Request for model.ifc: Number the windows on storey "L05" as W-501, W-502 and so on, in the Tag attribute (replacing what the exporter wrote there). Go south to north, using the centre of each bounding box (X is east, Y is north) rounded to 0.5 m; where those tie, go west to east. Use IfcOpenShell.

First a look at what the model holds.

```python
import ifcopenshell
import ifcopenshell.util.element
import ifcopenshell.util.placement

model = ifcopenshell.open("model.ifc")
print(model.schema)
storey = next(s for s in model.by_type("IfcBuildingStorey") if s.Name == "L05")
windows = [e for e in ifcopenshell.util.element.get_decomposition(storey) if e.is_a("IfcWindow")]
for e in sorted(windows, key=lambda e: e.id()):
    origin = ifcopenshell.util.placement.get_local_placement(e.ObjectPlacement)[:3, 3]
    print(e.id(), e.Tag, e.Name, origin.round(2) + 0.0, sep=" | ")
```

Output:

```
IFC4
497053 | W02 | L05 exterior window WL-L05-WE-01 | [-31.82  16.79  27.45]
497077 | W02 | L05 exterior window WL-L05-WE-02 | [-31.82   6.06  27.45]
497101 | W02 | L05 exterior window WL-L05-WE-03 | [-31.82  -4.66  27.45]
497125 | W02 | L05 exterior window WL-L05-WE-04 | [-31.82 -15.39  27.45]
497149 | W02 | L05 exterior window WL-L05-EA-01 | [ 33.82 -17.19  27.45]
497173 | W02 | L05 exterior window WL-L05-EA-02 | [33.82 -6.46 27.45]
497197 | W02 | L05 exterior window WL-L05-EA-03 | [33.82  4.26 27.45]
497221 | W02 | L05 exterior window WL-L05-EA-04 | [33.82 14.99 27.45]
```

```python
import ifcopenshell
import ifcopenshell.geom
import ifcopenshell.util.element
import ifcopenshell.util.shape

model = ifcopenshell.open("model.ifc")
settings = ifcopenshell.geom.settings()
settings.set("use-world-coords", True)


def centre(element):
    shape = ifcopenshell.geom.create_shape(settings, element)
    return ifcopenshell.util.shape.get_bbox_centroid(shape.geometry)


storey = next(s for s in model.by_type("IfcBuildingStorey") if s.Name == "L05")
windows = [e for e in ifcopenshell.util.element.get_decomposition(storey) if e.is_a("IfcWindow")]

# Insertion points can sit at a corner or the storey origin, so sort by the geometry (in metres).
centres = {e: centre(e) for e in windows}
windows.sort(key=lambda e: (round(centres[e][1] / 0.5), centres[e][0]))

for i, e in enumerate(windows, start=1):
    number = f"W-5{i:02d}"
    e.Tag = number
    print(e.id(), number)

model.write("model_v2.ifc")
```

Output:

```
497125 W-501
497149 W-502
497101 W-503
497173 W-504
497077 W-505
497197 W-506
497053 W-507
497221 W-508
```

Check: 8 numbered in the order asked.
